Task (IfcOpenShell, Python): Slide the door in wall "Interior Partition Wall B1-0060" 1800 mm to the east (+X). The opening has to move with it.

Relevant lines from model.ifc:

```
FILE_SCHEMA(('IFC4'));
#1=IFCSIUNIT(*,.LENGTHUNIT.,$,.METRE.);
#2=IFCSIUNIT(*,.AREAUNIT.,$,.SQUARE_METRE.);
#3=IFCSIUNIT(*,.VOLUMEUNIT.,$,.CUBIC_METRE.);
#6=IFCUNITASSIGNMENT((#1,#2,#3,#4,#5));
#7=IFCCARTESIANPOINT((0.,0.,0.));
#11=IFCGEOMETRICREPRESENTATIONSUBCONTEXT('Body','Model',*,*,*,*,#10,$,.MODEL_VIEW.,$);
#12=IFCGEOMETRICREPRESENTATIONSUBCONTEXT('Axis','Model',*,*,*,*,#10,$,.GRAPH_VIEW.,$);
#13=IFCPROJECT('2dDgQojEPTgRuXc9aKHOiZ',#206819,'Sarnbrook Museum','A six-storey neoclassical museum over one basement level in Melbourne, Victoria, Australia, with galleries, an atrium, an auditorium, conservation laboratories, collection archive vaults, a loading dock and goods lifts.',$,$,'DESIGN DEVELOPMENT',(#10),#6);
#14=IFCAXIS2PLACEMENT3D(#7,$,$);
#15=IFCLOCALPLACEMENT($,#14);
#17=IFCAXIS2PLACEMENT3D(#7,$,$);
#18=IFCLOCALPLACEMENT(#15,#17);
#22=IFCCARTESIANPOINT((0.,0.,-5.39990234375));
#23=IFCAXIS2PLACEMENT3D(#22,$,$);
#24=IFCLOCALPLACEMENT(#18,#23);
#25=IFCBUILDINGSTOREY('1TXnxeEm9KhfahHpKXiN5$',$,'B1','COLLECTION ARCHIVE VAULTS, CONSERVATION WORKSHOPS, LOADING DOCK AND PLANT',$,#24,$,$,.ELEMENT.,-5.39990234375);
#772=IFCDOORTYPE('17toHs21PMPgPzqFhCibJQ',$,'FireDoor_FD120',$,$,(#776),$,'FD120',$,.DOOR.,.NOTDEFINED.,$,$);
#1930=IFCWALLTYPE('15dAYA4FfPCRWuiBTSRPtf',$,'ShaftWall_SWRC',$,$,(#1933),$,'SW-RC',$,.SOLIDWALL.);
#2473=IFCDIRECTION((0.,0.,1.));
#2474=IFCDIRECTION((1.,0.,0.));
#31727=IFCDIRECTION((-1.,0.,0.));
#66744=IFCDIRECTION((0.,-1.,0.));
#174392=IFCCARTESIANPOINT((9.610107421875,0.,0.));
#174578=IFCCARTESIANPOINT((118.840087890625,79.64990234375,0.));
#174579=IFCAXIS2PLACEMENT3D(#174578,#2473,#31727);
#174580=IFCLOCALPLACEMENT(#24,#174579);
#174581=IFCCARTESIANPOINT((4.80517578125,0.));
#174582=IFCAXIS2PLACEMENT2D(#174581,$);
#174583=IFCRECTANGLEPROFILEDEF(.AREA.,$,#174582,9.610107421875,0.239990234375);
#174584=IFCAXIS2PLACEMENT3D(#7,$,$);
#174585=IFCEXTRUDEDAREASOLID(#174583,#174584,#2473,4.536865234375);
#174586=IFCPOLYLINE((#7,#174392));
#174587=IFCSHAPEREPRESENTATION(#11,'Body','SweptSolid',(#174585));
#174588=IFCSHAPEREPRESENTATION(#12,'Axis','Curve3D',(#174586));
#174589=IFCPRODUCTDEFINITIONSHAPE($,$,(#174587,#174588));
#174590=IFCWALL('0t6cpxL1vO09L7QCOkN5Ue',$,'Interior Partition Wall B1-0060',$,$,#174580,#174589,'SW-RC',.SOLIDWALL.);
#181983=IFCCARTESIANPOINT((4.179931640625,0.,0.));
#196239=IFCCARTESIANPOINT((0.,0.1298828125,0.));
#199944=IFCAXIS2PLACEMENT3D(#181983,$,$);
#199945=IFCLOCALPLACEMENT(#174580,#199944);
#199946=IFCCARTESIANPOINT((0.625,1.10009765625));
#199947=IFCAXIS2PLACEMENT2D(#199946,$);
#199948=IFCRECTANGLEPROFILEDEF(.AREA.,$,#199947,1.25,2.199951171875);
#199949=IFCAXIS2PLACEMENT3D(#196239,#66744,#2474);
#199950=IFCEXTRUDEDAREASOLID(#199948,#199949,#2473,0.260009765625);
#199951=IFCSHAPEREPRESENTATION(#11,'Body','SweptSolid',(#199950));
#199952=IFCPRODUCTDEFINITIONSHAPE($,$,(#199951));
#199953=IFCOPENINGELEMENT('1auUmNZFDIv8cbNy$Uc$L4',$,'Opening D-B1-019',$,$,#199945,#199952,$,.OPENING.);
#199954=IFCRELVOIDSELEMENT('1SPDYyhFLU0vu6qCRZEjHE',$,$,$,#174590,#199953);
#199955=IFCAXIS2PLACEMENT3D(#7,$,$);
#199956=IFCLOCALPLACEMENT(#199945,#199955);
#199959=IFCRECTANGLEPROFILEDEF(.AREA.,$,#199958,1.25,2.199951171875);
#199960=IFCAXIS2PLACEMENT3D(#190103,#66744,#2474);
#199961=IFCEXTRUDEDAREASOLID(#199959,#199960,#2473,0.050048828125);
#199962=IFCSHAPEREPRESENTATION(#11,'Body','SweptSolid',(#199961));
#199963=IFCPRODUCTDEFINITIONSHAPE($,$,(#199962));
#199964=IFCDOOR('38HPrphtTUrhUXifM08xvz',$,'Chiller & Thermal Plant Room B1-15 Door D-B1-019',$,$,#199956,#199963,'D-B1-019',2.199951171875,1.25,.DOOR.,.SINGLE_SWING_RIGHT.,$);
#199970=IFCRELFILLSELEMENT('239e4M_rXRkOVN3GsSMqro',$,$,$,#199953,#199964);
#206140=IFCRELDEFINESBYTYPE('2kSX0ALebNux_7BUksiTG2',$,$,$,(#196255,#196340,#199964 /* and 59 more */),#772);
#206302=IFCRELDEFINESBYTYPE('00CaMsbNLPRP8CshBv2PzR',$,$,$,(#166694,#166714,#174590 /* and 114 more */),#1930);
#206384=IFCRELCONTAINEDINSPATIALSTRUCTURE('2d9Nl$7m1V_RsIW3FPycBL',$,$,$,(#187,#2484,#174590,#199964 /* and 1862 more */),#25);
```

```python
import ifcopenshell
import ifcopenshell.api.geometry
import ifcopenshell.util.placement
import ifcopenshell.util.unit

model = ifcopenshell.open("model.ifc")
unit_scale = ifcopenshell.util.unit.calculate_unit_scale(model)

door = model.by_guid("38HPrphtTUrhUXifM08xvz")
opening = door.FillsVoids[0].RelatingOpeningElement
wall = opening.VoidsElements[0].RelatingBuildingElement

wall_matrix = ifcopenshell.util.placement.get_local_placement(wall.ObjectPlacement)
shift = wall_matrix[:3, 0] * -1.8 / unit_scale
before = ifcopenshell.util.placement.get_local_placement(door.ObjectPlacement)[:3, 3].copy()

# The door is placed relative to its opening, so it follows when the opening moves.
matrix = ifcopenshell.util.placement.get_local_placement(opening.ObjectPlacement)
matrix[:3, 3] += shift
ifcopenshell.api.geometry.edit_object_placement(
    model, product=opening, matrix=matrix, is_si=False, should_transform_children=True
)

after = ifcopenshell.util.placement.get_local_placement(door.ObjectPlacement)[:3, 3]
print("door moved by", (after - before).round(3) + 0.0)

model.write("model_edited.ifc")
```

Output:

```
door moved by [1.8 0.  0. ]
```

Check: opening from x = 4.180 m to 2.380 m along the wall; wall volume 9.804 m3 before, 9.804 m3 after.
